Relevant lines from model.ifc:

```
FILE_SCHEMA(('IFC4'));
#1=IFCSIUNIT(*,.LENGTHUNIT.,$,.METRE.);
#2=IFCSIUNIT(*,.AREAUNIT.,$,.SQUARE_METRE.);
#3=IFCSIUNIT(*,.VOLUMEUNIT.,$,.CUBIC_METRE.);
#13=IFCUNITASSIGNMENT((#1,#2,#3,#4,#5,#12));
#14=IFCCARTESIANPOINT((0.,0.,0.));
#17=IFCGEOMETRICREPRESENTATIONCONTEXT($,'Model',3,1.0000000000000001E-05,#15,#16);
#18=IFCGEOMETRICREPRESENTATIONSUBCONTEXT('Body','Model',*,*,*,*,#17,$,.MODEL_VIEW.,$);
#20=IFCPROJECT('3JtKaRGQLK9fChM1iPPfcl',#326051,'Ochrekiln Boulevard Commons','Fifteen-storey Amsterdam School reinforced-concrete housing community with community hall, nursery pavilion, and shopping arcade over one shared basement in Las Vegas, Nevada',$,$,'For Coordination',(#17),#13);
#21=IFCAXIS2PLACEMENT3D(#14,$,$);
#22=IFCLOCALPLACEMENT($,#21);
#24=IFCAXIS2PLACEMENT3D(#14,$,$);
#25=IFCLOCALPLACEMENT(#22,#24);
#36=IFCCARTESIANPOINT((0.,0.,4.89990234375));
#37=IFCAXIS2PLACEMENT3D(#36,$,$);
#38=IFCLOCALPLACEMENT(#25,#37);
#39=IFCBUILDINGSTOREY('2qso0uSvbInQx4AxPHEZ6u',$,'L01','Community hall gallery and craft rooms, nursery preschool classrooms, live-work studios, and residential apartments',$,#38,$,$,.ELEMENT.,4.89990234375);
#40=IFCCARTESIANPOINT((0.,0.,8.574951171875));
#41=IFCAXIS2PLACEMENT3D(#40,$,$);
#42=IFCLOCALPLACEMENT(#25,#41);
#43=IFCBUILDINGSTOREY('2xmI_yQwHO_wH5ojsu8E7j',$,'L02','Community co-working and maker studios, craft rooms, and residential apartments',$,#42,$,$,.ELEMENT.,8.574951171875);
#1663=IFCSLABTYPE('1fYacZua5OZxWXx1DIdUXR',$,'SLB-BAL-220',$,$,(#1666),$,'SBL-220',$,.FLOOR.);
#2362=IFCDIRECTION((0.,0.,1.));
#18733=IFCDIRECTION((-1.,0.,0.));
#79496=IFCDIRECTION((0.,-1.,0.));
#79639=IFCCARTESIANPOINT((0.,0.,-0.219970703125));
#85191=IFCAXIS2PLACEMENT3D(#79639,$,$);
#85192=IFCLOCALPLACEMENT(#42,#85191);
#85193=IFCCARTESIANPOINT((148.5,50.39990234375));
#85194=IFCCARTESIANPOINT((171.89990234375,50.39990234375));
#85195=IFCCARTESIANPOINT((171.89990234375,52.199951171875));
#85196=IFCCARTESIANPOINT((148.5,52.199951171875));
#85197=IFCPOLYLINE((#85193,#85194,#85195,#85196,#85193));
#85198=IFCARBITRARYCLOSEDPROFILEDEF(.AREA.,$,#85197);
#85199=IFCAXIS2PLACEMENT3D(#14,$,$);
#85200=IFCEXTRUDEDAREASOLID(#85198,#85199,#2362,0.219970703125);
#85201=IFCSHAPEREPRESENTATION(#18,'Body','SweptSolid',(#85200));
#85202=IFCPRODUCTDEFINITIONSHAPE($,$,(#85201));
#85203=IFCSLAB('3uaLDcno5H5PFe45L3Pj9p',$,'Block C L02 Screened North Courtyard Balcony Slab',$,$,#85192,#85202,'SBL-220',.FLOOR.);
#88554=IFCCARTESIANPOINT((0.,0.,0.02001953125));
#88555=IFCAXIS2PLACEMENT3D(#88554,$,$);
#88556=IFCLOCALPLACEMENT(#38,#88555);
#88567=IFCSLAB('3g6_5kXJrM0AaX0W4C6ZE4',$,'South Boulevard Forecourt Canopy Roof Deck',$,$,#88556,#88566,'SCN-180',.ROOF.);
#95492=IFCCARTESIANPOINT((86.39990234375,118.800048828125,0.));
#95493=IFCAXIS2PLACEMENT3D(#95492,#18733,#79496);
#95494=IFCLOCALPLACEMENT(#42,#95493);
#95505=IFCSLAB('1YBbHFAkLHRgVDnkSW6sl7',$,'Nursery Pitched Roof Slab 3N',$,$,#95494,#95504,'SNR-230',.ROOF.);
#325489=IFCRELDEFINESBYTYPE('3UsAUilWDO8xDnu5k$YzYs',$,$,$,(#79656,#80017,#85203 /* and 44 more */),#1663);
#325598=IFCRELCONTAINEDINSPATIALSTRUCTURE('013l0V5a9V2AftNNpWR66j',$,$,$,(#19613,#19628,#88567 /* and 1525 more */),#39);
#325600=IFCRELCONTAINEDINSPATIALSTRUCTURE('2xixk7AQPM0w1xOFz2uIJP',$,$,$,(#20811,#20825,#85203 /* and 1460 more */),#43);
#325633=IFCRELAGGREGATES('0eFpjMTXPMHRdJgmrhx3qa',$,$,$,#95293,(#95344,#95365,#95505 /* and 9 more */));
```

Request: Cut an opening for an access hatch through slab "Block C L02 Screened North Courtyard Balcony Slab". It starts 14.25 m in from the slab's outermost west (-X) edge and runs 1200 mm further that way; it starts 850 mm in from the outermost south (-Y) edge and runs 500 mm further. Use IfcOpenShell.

```python
import numpy as np
import ifcopenshell
import ifcopenshell.api.feature
import ifcopenshell.api.geometry
import ifcopenshell.api.root
import ifcopenshell.geom
import ifcopenshell.util.placement
import ifcopenshell.util.representation
import ifcopenshell.util.shape
import ifcopenshell.util.unit

model = ifcopenshell.open("model.ifc")
unit_scale = ifcopenshell.util.unit.calculate_unit_scale(model)
settings = ifcopenshell.geom.settings()


def volume(element):
    """Net volume in cubic metres, openings subtracted."""
    shape = ifcopenshell.geom.create_shape(settings, element)
    return ifcopenshell.util.shape.get_volume(shape.geometry)


slab = model.by_id(85203)
before = volume(slab)

# Extent in the slab's own axes, in metres. The edges named are its -X and -Y sides.
slab_shape = ifcopenshell.geom.create_shape(settings, slab)
vertices = ifcopenshell.util.shape.get_vertices(slab_shape.geometry)
x_min, y_min, bottom = vertices.min(axis=0)
top = vertices[:, 2].max()

opening = ifcopenshell.api.root.create_entity(model, ifc_class="IfcOpeningElement", name="Access hatch opening", predefined_type="OPENING")
context = ifcopenshell.util.representation.get_context(model, "Model", "Body", "MODEL_VIEW")
width, depth = 1.2, 0.5
outline = [(0.0, 0.0), (width, 0.0), (width, depth), (0.0, depth), (0.0, 0.0)]
# Overshoot both faces by 50 mm so the cut is clean.
shape = ifcopenshell.api.geometry.add_slab_representation(
    model, context=context, depth=top - bottom + 0.1, polyline=outline
)
ifcopenshell.api.geometry.assign_representation(model, product=opening, representation=shape)

matrix = ifcopenshell.util.placement.get_local_placement(slab.ObjectPlacement)
matrix[:, 3] = matrix @ np.append(np.array([x_min + 14.25, y_min + 0.85, bottom - 0.05]) / unit_scale, 1.0)
ifcopenshell.api.geometry.edit_object_placement(model, product=opening, matrix=matrix, is_si=False)
ifcopenshell.api.feature.add_feature(model, feature=opening, element=slab)

after = volume(slab)

print(f"slab volume {before:.3f} -> {after:.3f} m3")

model.write("model_v2.ifc")
```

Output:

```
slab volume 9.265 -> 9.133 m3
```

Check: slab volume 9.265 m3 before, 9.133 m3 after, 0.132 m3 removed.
